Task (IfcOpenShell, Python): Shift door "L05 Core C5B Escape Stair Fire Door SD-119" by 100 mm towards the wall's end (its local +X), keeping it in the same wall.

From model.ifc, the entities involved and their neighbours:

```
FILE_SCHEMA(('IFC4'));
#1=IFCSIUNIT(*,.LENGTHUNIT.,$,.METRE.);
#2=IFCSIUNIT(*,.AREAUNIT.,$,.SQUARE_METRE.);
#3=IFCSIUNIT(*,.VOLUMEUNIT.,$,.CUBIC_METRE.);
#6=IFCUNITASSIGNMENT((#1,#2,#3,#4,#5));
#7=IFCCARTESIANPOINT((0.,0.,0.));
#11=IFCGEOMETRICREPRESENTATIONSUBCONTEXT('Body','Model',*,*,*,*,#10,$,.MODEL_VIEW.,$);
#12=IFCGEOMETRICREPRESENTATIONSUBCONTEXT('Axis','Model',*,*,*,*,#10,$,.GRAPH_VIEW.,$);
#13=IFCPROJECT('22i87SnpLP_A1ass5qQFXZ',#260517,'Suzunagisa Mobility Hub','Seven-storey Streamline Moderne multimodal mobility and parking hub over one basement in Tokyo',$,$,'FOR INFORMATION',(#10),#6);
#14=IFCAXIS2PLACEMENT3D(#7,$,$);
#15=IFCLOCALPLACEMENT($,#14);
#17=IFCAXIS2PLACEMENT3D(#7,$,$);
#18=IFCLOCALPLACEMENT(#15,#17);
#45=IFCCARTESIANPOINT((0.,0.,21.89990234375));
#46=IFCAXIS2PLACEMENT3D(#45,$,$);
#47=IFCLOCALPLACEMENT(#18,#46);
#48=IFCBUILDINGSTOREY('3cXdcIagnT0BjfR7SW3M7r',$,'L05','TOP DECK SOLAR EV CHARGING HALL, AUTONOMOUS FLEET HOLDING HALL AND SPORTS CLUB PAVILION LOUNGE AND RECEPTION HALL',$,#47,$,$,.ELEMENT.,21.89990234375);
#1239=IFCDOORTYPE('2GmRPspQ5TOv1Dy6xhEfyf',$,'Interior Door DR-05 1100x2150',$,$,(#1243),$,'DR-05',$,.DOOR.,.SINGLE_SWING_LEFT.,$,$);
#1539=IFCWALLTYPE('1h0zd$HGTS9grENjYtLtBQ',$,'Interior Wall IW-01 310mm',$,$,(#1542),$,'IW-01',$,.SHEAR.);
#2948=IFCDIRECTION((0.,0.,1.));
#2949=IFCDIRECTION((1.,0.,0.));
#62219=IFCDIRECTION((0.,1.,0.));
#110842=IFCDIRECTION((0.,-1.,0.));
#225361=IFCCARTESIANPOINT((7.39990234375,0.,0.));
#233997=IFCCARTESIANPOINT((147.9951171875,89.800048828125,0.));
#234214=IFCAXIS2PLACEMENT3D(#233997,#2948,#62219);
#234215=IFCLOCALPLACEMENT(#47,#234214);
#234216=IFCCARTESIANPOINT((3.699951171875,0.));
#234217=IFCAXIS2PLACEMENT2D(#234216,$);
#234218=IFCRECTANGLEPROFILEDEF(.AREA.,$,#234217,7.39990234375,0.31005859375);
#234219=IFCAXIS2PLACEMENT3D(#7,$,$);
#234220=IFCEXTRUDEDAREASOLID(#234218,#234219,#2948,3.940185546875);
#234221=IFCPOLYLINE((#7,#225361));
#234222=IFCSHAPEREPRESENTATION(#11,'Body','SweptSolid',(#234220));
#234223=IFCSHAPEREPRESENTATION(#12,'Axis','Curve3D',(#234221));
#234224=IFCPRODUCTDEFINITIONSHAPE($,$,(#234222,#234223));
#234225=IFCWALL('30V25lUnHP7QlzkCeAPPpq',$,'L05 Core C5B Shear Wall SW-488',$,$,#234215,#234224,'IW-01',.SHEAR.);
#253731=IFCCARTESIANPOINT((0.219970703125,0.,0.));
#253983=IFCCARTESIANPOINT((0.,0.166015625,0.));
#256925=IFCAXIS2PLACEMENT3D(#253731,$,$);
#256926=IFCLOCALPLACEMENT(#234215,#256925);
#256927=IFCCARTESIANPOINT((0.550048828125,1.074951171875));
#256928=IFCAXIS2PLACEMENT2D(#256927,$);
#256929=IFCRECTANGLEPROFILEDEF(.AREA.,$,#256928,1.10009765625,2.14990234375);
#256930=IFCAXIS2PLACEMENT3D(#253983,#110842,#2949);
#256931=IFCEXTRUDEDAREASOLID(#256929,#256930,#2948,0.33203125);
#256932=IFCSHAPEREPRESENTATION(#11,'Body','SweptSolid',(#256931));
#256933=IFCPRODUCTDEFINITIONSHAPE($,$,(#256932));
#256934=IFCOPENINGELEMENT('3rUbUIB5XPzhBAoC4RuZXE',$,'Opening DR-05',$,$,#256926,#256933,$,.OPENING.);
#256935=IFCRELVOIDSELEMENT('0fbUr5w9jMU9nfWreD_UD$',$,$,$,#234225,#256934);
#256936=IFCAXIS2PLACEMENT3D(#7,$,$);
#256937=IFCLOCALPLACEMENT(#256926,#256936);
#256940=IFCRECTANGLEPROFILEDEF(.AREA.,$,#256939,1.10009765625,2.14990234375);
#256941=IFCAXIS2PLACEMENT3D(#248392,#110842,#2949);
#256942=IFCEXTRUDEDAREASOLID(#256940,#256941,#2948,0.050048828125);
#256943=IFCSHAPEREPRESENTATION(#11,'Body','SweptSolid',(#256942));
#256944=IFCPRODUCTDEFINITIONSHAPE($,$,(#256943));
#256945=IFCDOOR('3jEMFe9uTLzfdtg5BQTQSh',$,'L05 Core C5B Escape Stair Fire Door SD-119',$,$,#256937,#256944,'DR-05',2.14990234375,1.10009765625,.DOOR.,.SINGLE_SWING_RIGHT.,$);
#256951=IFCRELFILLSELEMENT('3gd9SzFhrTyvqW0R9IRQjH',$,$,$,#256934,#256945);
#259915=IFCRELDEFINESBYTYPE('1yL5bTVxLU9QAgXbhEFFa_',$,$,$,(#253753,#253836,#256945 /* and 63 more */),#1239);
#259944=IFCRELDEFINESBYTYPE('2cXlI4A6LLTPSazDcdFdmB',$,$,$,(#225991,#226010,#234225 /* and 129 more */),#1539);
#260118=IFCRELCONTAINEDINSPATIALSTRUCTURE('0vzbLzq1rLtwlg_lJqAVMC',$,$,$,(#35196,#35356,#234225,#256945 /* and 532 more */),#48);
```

```python
import ifcopenshell
import ifcopenshell.api.geometry
import ifcopenshell.util.placement
import ifcopenshell.util.unit

model = ifcopenshell.open("model.ifc")
unit_scale = ifcopenshell.util.unit.calculate_unit_scale(model)

door = model.by_id(256945)
opening = door.FillsVoids[0].RelatingOpeningElement
wall = opening.VoidsElements[0].RelatingBuildingElement

wall_matrix = ifcopenshell.util.placement.get_local_placement(wall.ObjectPlacement)
shift = wall_matrix[:3, 0] * 0.1 / unit_scale
before = ifcopenshell.util.placement.get_local_placement(door.ObjectPlacement)[:3, 3].copy()

# The door is placed relative to its opening, so it follows when the opening moves.
matrix = ifcopenshell.util.placement.get_local_placement(opening.ObjectPlacement)
matrix[:3, 3] += shift
ifcopenshell.api.geometry.edit_object_placement(
    model, product=opening, matrix=matrix, is_si=False, should_transform_children=True
)

after = ifcopenshell.util.placement.get_local_placement(door.ObjectPlacement)[:3, 3]
print("door moved by", (after - before).round(3) + 0.0)

model.write("model_edited.ifc")
```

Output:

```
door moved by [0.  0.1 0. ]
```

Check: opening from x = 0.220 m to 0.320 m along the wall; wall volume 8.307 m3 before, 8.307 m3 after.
